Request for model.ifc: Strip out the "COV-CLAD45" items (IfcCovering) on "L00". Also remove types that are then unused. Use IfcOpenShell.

First a look at what the model holds.

```python
import ifcopenshell
import ifcopenshell.util.element

model = ifcopenshell.open("model.ifc")
print(model.schema)
storey = next(s for s in model.by_type("IfcBuildingStorey") if s.Name == "L00")
coverings = [e for e in ifcopenshell.util.element.get_decomposition(storey) if e.is_a("IfcCovering")]
seen = {}
for e in coverings:
    element_type = ifcopenshell.util.element.get_type(e)
    name = element_type.Name if element_type not in (None, e) else None
    seen[name] = seen.get(name, 0) + 1
for name, count in sorted(seen.items(), key=str):
    print(count, "x", name)
```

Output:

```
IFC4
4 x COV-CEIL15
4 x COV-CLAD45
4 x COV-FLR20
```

```python
import ifcopenshell
import ifcopenshell.api.root
import ifcopenshell.util.element

model = ifcopenshell.open("model.ifc")

storey = next(s for s in model.by_type("IfcBuildingStorey") if s.Name == "L00")
coverings = [e for e in ifcopenshell.util.element.get_decomposition(storey) if e.is_a("IfcCovering")]
targets = [e for e in coverings if (t := ifcopenshell.util.element.get_type(e)) not in (None, e) and t.Name == "COV-CLAD45"]
types = {ifcopenshell.util.element.get_type(e) for e in targets} - {None, *targets}

for e in targets:
    ifcopenshell.api.root.remove_product(model, product=e)
print(len(targets), "removed")

unused = [t for t in types if not ifcopenshell.util.element.get_types(t)]
for t in unused:
    ifcopenshell.api.root.remove_product(model, product=t)
print(len(unused), "unused types removed")

model.write("model_updated.ifc")
```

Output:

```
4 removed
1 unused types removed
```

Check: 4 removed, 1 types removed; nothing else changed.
